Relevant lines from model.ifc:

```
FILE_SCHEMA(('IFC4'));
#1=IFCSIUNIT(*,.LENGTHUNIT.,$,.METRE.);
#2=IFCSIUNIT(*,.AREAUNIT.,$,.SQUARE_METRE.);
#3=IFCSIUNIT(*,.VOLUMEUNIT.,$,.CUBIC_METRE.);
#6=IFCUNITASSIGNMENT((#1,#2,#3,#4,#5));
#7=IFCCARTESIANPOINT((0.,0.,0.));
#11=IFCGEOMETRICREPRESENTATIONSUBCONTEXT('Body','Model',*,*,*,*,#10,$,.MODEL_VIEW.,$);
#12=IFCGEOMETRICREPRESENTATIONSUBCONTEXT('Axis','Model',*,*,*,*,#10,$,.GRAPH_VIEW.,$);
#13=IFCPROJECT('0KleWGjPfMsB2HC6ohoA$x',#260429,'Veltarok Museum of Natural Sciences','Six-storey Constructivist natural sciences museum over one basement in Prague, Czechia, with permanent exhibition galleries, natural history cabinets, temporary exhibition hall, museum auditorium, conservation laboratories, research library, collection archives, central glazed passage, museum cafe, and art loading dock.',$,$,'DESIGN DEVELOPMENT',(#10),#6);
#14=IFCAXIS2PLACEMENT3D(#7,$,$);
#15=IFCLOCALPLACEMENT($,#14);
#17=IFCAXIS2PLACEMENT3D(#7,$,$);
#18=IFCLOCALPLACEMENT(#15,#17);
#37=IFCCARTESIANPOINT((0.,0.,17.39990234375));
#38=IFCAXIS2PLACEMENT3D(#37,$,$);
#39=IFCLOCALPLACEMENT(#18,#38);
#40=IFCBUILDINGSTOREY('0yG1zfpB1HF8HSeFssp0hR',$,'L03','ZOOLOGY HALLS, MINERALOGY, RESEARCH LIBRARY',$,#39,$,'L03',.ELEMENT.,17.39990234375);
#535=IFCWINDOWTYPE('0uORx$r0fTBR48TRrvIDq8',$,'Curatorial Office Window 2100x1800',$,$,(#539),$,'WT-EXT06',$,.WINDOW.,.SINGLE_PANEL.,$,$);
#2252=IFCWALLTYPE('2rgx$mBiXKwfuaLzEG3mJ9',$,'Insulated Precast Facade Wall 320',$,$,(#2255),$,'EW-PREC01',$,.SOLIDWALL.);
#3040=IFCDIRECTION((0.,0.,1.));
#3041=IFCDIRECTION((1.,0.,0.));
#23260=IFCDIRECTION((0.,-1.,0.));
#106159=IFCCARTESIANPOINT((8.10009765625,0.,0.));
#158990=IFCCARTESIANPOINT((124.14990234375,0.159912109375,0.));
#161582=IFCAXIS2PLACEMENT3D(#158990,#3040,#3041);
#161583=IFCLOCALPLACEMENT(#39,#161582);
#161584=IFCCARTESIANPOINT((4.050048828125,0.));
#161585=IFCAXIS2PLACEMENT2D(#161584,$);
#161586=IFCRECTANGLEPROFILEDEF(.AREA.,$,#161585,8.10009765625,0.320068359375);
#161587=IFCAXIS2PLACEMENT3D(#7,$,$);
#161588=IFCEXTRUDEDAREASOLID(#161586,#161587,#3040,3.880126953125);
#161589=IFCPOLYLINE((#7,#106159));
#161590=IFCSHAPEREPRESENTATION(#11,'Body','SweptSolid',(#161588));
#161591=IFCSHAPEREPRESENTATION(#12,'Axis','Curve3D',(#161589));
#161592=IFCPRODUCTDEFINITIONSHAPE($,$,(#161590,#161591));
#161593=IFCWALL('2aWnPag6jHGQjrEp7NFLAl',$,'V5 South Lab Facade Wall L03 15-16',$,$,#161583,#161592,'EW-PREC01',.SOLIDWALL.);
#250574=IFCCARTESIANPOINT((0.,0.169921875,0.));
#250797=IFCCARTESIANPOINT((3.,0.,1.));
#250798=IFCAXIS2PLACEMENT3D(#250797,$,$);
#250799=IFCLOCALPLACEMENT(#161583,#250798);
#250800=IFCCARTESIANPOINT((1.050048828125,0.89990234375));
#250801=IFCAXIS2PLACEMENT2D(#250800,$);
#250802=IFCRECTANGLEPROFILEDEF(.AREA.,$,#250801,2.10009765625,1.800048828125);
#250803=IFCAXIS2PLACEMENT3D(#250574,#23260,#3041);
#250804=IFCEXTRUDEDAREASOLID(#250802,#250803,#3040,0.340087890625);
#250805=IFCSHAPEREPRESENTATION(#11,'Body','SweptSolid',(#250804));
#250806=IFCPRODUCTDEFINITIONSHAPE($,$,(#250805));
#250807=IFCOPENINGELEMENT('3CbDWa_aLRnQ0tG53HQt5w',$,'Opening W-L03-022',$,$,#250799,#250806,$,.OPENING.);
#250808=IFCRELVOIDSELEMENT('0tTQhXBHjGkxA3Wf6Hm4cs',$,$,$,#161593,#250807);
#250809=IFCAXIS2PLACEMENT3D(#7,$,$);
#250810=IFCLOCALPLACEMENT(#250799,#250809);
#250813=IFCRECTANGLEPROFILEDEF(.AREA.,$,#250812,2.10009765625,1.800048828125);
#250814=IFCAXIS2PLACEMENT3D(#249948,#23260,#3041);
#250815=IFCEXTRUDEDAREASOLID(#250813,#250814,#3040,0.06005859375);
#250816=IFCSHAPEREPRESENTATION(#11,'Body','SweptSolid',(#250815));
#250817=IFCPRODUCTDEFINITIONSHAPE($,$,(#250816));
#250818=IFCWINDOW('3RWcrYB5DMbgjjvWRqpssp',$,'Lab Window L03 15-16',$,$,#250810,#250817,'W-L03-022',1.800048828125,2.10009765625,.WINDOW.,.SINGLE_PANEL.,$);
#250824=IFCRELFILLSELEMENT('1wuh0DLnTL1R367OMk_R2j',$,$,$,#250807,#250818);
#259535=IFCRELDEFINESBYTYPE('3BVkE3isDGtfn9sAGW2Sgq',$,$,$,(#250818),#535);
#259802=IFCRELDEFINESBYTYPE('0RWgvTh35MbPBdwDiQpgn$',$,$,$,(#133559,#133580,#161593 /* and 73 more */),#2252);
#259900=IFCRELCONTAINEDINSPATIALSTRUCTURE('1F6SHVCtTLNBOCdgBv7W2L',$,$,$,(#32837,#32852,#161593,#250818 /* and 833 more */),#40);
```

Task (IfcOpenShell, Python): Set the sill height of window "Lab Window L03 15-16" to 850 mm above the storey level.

```python
import numpy as np
import ifcopenshell
import ifcopenshell.api.geometry
import ifcopenshell.geom
import ifcopenshell.util.element
import ifcopenshell.util.placement
import ifcopenshell.util.shape
import ifcopenshell.util.unit

model = ifcopenshell.open("model.ifc")
unit_scale = ifcopenshell.util.unit.calculate_unit_scale(model)

window = model.by_guid("3RWcrYB5DMbgjjvWRqpssp")
opening = window.FillsVoids[0].RelatingOpeningElement
storey = ifcopenshell.util.element.get_container(window, ifc_class="IfcBuildingStorey")
level = ifcopenshell.util.placement.get_local_placement(storey.ObjectPlacement)[2, 3]

# The opening's origin need not be at the sill, so measure its lowest point.
shape = ifcopenshell.geom.create_shape(ifcopenshell.geom.settings(), opening)
bottom = ifcopenshell.util.shape.get_shape_bottom_elevation(shape, shape.geometry) / unit_scale
dz = level + 0.85 - bottom

shift = np.array([0.0, 0.0, dz])
# The window is placed relative to its opening, so it follows when the opening moves.
matrix = ifcopenshell.util.placement.get_local_placement(opening.ObjectPlacement)
matrix[:3, 3] += shift
ifcopenshell.api.geometry.edit_object_placement(
    model, product=opening, matrix=matrix, is_si=False, should_transform_children=True
)

print(f"moved by {dz * unit_scale:+.3f} m")

model.write("model_rev.ifc")
```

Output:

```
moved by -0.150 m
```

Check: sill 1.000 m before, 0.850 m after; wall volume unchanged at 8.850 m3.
